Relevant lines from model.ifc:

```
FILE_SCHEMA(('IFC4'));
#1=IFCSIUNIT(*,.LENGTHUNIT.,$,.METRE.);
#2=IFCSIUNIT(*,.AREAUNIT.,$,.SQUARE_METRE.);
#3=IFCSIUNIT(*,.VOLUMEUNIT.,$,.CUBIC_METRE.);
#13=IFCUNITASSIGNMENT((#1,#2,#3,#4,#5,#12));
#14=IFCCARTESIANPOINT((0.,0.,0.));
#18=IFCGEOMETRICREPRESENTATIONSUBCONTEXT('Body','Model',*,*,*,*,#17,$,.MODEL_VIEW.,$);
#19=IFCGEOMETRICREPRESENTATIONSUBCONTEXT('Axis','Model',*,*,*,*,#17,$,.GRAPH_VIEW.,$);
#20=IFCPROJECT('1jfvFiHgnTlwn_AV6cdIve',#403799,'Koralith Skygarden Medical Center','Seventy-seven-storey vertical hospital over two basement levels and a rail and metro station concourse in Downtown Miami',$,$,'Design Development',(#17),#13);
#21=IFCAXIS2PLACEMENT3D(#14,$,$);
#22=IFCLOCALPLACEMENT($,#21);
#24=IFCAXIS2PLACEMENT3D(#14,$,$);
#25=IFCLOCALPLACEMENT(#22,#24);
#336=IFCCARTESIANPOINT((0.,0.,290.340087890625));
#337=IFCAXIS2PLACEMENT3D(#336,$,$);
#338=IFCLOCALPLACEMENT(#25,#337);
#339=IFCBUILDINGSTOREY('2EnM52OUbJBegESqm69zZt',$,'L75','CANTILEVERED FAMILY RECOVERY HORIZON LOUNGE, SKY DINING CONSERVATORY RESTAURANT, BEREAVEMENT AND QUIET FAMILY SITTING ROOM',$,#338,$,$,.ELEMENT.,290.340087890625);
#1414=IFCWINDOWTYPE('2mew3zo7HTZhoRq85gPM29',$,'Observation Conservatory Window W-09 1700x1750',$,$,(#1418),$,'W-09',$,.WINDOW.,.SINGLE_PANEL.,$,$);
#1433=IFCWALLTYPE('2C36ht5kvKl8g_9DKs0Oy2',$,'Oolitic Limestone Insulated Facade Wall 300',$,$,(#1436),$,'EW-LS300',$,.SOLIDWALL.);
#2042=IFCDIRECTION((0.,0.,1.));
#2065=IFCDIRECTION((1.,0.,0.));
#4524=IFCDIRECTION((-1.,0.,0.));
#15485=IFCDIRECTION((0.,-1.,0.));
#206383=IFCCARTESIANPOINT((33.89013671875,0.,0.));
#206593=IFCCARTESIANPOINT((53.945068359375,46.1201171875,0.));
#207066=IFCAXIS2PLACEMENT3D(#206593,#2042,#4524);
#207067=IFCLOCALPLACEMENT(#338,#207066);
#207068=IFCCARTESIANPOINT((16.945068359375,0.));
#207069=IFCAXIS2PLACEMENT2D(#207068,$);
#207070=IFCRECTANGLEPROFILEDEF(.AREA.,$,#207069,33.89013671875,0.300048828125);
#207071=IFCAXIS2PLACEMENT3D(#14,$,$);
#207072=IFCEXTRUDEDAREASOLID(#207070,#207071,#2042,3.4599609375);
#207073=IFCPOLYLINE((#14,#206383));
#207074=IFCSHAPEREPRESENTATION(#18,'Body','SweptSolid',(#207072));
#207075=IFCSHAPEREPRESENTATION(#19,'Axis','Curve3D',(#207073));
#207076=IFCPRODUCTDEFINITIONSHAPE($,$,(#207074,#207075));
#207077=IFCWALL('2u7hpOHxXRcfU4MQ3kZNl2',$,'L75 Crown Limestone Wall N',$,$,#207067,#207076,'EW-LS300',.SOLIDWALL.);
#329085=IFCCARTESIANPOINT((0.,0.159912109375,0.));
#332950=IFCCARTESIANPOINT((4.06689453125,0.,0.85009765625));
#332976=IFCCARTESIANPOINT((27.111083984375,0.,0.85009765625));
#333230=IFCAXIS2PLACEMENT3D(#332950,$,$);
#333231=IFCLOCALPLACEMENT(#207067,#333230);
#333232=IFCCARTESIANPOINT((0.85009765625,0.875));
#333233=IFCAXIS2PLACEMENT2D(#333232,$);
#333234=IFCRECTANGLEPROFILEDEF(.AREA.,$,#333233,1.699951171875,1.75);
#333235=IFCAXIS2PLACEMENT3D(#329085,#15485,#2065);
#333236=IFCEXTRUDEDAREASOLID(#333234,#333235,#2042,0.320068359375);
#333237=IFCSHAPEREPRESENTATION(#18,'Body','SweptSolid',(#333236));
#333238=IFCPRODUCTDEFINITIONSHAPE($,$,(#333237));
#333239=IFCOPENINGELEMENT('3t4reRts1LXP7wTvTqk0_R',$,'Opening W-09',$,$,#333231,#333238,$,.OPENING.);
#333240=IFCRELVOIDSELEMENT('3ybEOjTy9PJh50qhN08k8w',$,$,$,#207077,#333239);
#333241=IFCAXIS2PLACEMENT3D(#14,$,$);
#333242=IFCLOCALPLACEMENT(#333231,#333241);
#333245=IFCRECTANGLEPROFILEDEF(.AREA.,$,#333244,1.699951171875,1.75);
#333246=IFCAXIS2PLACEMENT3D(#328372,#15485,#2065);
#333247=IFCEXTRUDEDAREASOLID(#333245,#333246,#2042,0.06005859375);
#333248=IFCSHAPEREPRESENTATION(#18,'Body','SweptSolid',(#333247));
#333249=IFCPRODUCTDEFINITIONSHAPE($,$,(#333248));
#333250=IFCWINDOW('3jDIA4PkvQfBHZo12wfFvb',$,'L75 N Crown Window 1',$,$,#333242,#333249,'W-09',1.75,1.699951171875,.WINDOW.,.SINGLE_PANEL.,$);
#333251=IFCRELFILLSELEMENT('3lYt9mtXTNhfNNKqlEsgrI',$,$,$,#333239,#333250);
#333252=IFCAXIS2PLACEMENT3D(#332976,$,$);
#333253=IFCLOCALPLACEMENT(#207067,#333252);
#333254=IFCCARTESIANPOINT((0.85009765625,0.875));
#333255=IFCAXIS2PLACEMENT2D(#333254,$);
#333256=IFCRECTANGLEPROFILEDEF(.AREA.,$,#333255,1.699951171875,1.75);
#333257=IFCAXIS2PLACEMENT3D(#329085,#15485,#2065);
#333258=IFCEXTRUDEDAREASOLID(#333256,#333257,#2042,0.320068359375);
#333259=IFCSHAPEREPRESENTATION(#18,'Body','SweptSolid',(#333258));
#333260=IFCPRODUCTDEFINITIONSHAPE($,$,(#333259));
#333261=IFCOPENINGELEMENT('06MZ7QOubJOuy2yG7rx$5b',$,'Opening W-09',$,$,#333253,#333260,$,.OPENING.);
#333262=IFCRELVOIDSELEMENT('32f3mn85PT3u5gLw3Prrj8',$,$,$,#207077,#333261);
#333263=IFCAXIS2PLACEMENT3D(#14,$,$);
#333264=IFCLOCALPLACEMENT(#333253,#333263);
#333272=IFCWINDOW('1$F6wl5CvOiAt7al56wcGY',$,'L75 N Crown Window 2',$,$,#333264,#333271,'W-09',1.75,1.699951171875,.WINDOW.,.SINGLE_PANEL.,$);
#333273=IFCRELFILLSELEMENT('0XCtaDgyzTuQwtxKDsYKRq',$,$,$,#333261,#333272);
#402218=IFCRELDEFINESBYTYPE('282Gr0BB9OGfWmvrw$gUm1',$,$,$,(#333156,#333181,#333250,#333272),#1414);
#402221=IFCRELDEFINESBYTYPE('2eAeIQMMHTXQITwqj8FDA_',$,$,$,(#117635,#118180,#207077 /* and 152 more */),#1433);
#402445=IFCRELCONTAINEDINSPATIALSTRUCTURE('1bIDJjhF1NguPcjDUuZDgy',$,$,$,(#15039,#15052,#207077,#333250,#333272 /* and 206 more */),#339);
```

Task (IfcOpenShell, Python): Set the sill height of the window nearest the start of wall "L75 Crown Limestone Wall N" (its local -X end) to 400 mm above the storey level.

```python
import numpy as np
import ifcopenshell
import ifcopenshell.api.geometry
import ifcopenshell.geom
import ifcopenshell.util.element
import ifcopenshell.util.placement
import ifcopenshell.util.shape
import ifcopenshell.util.unit

model = ifcopenshell.open("model.ifc")
unit_scale = ifcopenshell.util.unit.calculate_unit_scale(model)

window = model.by_guid("3jDIA4PkvQfBHZo12wfFvb")
opening = window.FillsVoids[0].RelatingOpeningElement
storey = ifcopenshell.util.element.get_container(window, ifc_class="IfcBuildingStorey")
level = ifcopenshell.util.placement.get_local_placement(storey.ObjectPlacement)[2, 3]

# The opening's origin need not be at the sill, so measure its lowest point.
shape = ifcopenshell.geom.create_shape(ifcopenshell.geom.settings(), opening)
bottom = ifcopenshell.util.shape.get_shape_bottom_elevation(shape, shape.geometry) / unit_scale
dz = level + 0.4 - bottom

shift = np.array([0.0, 0.0, dz])
# The window is placed relative to its opening, so it follows when the opening moves.
matrix = ifcopenshell.util.placement.get_local_placement(opening.ObjectPlacement)
matrix[:3, 3] += shift
ifcopenshell.api.geometry.edit_object_placement(
    model, product=opening, matrix=matrix, is_si=False, should_transform_children=True
)

print(f"moved by {dz * unit_scale:+.3f} m")

model.write("model_edited.ifc")
```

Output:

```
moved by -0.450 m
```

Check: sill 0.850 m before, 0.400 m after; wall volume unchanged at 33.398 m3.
